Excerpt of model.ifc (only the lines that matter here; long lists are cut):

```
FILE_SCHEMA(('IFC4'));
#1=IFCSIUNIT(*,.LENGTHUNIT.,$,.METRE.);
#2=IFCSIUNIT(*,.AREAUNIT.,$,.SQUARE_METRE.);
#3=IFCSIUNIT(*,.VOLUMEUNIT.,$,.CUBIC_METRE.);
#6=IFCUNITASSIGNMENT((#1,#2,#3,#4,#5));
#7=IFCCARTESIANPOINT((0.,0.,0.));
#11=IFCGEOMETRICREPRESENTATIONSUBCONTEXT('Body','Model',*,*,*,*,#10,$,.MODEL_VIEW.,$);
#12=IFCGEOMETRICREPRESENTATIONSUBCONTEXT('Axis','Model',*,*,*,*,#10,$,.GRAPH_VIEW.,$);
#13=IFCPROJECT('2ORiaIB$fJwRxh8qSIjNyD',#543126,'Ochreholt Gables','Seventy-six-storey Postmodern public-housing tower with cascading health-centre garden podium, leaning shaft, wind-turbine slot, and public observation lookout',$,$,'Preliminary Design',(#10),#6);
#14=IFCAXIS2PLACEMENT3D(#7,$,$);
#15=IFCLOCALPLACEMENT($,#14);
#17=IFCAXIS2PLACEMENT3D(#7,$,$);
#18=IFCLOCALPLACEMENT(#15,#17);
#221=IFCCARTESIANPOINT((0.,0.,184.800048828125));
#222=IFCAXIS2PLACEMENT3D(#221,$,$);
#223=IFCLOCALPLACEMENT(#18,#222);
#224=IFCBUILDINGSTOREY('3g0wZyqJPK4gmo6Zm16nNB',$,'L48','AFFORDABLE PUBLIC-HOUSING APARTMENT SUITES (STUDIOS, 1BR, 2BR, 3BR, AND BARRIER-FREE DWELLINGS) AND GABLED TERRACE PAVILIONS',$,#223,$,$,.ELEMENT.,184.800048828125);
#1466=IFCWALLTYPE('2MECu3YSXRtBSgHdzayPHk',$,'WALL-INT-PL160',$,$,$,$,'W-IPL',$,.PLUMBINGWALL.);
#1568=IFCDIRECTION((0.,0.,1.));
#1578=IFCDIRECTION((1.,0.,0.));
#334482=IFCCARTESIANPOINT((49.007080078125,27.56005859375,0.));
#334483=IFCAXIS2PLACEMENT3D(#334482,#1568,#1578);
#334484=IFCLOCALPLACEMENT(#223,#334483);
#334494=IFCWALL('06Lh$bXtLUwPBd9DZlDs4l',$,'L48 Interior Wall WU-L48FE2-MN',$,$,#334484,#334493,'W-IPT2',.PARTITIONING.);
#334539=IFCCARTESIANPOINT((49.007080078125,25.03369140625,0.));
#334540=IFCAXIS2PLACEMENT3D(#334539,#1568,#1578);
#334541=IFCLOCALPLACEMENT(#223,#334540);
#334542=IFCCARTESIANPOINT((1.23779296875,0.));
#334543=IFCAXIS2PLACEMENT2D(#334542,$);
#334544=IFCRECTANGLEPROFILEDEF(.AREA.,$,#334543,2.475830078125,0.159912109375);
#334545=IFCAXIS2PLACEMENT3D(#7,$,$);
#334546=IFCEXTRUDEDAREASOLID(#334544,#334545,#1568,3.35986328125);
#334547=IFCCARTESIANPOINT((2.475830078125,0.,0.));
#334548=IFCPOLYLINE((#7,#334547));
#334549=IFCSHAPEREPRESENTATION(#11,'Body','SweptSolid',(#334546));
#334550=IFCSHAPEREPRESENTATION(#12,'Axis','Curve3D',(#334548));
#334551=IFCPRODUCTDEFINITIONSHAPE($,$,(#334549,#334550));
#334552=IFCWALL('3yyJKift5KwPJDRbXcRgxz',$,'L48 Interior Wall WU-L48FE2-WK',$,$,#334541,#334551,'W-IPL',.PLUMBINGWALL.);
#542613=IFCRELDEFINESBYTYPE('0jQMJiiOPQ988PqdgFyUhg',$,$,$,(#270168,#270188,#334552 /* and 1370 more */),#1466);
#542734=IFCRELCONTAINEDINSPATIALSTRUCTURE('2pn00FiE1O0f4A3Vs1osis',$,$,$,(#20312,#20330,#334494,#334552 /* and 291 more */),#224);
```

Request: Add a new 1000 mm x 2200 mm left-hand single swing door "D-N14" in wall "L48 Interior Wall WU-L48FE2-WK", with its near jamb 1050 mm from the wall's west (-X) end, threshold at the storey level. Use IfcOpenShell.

```python
import numpy as np
import ifcopenshell
import ifcopenshell.api.feature
import ifcopenshell.api.geometry
import ifcopenshell.api.root
import ifcopenshell.api.spatial
import ifcopenshell.geom
import ifcopenshell.util.element
import ifcopenshell.util.placement
import ifcopenshell.util.representation
import ifcopenshell.util.shape
import ifcopenshell.util.unit

model = ifcopenshell.open("model.ifc")
unit_scale = ifcopenshell.util.unit.calculate_unit_scale(model)
settings = ifcopenshell.geom.settings()


def volume(element):
    """Net volume in cubic metres, openings subtracted."""
    shape = ifcopenshell.geom.create_shape(settings, element)
    return ifcopenshell.util.shape.get_volume(shape.geometry)


wall = model.by_guid("3yyJKift5KwPJDRbXcRgxz")
storey = ifcopenshell.util.element.get_container(wall, ifc_class="IfcBuildingStorey")
context = ifcopenshell.util.representation.get_context(model, "Model", "Body", "MODEL_VIEW")
before = volume(wall)

width, height, from_end, sill = 1, 2.2, 1.05, 0.0  # metres

# The wall runs along its own X axis, and the end named is its -X end.
wall_shape = ifcopenshell.geom.create_shape(settings, wall)
x, y, z = ifcopenshell.util.shape.get_vertices(wall_shape.geometry).T
start = x.min() + from_end
face, thickness = float(y.min()), float(y.max() - y.min())
wall_matrix = ifcopenshell.util.placement.get_local_placement(wall.ObjectPlacement)
level = ifcopenshell.util.placement.get_local_placement(storey.ObjectPlacement)[2, 3]


def in_wall(x, y):
    """Placement at x, y metres in the wall's axes, at sill height."""
    matrix = wall_matrix.copy()
    matrix[:, 3] = wall_matrix @ np.array([x / unit_scale, y / unit_scale, 0.0, 1.0])
    matrix[2, 3] = level + sill / unit_scale
    return matrix


# Opening: a box that overshoots both wall faces by 50 mm.
opening = ifcopenshell.api.root.create_entity(model, ifc_class="IfcOpeningElement", predefined_type="OPENING")
box = ifcopenshell.api.geometry.add_wall_representation(
    model, context=context, length=width, height=height, thickness=thickness + 0.1
)
ifcopenshell.api.geometry.assign_representation(model, product=opening, representation=box)
ifcopenshell.api.geometry.edit_object_placement(model, product=opening, matrix=in_wall(start, face - 0.05), is_si=False)
ifcopenshell.api.feature.add_feature(model, feature=opening, element=wall)

door = ifcopenshell.api.root.create_entity(model, ifc_class="IfcDoor", name="D-N14", predefined_type="DOOR")
door.OverallWidth, door.OverallHeight = width / unit_scale, height / unit_scale
door.OperationType = "SINGLE_SWING_LEFT"
body = ifcopenshell.api.geometry.add_door_representation(
    model,
    context=context,
    overall_width=door.OverallWidth,
    overall_height=door.OverallHeight,
    operation_type="SINGLE_SWING_LEFT",
    lining_properties={"LiningDepth": thickness / unit_scale, "ThresholdDepth": thickness / unit_scale},
)
ifcopenshell.api.geometry.assign_representation(model, product=door, representation=body)
ifcopenshell.api.spatial.assign_container(model, products=[door], relating_structure=storey)
ifcopenshell.api.feature.add_filling(model, opening=opening, element=door)

# The lining spans the wall, so the door starts at the wall face.
ifcopenshell.api.geometry.edit_object_placement(model, product=door, matrix=in_wall(start, face), is_si=False)

after = volume(wall)

print(f"wall volume {before:.3f} -> {after:.3f} m3")

model.write("model_v2.ifc")
```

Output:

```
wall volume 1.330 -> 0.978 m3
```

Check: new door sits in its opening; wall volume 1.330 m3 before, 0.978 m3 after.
